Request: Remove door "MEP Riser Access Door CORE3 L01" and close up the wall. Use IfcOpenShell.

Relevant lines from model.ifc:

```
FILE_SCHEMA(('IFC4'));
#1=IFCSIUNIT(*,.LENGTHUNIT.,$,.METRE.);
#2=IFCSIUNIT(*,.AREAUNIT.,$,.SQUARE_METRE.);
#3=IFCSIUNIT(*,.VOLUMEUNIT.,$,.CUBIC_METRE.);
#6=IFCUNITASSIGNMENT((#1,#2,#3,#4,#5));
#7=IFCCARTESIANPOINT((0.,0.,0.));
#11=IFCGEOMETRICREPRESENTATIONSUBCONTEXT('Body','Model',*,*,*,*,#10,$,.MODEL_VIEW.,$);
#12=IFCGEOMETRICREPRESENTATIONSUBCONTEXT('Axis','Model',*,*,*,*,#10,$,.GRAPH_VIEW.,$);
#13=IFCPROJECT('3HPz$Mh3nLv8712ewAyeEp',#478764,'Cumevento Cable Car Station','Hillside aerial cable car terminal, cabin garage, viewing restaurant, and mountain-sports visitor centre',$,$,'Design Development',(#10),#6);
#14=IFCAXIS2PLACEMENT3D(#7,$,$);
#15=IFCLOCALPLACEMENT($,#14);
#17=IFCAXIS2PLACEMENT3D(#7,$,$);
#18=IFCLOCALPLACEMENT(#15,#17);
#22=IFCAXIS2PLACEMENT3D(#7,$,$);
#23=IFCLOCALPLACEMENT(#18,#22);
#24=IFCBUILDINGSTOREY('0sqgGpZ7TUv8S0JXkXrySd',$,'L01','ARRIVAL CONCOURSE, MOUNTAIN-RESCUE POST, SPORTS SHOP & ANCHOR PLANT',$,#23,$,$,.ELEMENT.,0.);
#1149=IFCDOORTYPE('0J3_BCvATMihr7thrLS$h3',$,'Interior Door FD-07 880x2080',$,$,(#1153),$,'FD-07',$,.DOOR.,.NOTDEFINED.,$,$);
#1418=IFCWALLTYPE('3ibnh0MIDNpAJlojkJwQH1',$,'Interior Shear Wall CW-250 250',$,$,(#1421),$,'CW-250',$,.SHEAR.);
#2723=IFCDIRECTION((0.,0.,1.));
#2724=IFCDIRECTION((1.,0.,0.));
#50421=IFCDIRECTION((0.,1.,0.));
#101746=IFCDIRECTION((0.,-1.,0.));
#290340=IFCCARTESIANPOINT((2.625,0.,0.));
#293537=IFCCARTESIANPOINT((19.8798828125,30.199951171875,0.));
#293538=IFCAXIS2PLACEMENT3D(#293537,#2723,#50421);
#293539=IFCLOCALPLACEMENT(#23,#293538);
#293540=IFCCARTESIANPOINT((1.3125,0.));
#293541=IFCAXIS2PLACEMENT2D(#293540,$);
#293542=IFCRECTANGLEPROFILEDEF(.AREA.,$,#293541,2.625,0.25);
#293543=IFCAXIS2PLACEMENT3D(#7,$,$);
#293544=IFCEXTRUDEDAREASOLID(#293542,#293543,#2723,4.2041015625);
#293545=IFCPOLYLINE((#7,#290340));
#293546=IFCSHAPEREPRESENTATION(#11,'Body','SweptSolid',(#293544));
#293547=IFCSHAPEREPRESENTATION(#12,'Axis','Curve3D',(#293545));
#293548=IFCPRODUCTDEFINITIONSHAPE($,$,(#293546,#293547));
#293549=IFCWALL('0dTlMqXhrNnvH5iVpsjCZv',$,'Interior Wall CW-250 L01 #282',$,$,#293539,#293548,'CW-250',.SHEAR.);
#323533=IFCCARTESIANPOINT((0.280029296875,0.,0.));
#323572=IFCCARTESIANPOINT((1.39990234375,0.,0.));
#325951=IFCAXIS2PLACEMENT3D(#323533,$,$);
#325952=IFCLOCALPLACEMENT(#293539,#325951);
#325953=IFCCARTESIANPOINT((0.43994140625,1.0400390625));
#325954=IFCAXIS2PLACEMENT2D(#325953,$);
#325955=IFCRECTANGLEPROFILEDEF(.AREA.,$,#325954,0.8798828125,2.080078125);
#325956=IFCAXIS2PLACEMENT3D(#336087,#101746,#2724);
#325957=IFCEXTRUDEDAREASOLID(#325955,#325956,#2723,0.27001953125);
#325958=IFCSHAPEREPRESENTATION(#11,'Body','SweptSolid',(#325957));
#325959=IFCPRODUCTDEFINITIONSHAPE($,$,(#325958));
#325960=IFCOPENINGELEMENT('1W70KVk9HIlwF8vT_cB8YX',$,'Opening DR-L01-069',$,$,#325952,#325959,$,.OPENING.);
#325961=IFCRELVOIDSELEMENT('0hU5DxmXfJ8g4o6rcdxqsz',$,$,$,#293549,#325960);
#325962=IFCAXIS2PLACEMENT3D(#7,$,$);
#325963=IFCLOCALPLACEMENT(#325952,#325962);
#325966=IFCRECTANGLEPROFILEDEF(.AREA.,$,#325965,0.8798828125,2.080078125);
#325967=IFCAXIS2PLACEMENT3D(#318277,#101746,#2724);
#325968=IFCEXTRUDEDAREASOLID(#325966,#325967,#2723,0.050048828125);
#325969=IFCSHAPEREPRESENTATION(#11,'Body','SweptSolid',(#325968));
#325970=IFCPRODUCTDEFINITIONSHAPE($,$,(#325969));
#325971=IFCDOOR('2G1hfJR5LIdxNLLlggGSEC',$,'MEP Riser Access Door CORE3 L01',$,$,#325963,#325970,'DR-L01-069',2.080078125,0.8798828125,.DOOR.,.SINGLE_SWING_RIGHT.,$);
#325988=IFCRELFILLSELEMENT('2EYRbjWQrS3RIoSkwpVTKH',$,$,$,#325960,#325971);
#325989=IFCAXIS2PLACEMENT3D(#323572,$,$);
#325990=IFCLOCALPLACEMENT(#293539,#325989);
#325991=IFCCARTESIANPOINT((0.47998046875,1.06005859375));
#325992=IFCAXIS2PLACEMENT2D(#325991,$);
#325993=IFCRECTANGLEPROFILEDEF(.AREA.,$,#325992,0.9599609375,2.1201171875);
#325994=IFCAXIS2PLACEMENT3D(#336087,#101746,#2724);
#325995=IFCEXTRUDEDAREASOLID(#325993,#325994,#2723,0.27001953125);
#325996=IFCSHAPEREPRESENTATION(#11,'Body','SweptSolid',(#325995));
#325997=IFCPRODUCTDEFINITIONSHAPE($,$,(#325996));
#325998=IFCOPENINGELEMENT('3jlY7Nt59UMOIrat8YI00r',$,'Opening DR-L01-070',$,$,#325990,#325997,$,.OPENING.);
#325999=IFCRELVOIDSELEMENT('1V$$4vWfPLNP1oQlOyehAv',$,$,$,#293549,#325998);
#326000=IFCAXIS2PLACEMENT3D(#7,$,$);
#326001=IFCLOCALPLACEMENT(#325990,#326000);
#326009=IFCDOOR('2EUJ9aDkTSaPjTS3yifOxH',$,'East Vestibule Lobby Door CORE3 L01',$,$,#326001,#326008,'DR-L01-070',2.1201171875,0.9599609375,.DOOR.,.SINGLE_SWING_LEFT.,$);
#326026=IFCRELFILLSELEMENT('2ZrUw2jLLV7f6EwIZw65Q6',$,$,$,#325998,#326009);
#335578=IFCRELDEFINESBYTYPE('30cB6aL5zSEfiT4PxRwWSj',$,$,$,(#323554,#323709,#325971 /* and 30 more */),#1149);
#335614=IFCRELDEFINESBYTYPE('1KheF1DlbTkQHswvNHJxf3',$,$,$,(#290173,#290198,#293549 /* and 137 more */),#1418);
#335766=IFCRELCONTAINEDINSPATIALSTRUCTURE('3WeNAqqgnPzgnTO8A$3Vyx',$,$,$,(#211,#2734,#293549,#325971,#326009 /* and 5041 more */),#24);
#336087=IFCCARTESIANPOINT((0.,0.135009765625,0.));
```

```python
import ifcopenshell
import ifcopenshell.api.feature
import ifcopenshell.api.root
import ifcopenshell.geom
import ifcopenshell.util.shape

model = ifcopenshell.open("model.ifc")
settings = ifcopenshell.geom.settings()


def volume(element):
    """Net volume in cubic metres, openings subtracted."""
    shape = ifcopenshell.geom.create_shape(settings, element)
    return ifcopenshell.util.shape.get_volume(shape.geometry)


door = model.by_guid("2G1hfJR5LIdxNLLlggGSEC")
opening = door.FillsVoids[0].RelatingOpeningElement
wall = opening.VoidsElements[0].RelatingBuildingElement
before = volume(wall)

ifcopenshell.api.root.remove_product(model, product=door)
ifcopenshell.api.feature.remove_feature(model, feature=opening)

after = volume(wall)

print(f"wall volume {before:.3f} -> {after:.3f} m3")

model.write("model_v2.ifc")
```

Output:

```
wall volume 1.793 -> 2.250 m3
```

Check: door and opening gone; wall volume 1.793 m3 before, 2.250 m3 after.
